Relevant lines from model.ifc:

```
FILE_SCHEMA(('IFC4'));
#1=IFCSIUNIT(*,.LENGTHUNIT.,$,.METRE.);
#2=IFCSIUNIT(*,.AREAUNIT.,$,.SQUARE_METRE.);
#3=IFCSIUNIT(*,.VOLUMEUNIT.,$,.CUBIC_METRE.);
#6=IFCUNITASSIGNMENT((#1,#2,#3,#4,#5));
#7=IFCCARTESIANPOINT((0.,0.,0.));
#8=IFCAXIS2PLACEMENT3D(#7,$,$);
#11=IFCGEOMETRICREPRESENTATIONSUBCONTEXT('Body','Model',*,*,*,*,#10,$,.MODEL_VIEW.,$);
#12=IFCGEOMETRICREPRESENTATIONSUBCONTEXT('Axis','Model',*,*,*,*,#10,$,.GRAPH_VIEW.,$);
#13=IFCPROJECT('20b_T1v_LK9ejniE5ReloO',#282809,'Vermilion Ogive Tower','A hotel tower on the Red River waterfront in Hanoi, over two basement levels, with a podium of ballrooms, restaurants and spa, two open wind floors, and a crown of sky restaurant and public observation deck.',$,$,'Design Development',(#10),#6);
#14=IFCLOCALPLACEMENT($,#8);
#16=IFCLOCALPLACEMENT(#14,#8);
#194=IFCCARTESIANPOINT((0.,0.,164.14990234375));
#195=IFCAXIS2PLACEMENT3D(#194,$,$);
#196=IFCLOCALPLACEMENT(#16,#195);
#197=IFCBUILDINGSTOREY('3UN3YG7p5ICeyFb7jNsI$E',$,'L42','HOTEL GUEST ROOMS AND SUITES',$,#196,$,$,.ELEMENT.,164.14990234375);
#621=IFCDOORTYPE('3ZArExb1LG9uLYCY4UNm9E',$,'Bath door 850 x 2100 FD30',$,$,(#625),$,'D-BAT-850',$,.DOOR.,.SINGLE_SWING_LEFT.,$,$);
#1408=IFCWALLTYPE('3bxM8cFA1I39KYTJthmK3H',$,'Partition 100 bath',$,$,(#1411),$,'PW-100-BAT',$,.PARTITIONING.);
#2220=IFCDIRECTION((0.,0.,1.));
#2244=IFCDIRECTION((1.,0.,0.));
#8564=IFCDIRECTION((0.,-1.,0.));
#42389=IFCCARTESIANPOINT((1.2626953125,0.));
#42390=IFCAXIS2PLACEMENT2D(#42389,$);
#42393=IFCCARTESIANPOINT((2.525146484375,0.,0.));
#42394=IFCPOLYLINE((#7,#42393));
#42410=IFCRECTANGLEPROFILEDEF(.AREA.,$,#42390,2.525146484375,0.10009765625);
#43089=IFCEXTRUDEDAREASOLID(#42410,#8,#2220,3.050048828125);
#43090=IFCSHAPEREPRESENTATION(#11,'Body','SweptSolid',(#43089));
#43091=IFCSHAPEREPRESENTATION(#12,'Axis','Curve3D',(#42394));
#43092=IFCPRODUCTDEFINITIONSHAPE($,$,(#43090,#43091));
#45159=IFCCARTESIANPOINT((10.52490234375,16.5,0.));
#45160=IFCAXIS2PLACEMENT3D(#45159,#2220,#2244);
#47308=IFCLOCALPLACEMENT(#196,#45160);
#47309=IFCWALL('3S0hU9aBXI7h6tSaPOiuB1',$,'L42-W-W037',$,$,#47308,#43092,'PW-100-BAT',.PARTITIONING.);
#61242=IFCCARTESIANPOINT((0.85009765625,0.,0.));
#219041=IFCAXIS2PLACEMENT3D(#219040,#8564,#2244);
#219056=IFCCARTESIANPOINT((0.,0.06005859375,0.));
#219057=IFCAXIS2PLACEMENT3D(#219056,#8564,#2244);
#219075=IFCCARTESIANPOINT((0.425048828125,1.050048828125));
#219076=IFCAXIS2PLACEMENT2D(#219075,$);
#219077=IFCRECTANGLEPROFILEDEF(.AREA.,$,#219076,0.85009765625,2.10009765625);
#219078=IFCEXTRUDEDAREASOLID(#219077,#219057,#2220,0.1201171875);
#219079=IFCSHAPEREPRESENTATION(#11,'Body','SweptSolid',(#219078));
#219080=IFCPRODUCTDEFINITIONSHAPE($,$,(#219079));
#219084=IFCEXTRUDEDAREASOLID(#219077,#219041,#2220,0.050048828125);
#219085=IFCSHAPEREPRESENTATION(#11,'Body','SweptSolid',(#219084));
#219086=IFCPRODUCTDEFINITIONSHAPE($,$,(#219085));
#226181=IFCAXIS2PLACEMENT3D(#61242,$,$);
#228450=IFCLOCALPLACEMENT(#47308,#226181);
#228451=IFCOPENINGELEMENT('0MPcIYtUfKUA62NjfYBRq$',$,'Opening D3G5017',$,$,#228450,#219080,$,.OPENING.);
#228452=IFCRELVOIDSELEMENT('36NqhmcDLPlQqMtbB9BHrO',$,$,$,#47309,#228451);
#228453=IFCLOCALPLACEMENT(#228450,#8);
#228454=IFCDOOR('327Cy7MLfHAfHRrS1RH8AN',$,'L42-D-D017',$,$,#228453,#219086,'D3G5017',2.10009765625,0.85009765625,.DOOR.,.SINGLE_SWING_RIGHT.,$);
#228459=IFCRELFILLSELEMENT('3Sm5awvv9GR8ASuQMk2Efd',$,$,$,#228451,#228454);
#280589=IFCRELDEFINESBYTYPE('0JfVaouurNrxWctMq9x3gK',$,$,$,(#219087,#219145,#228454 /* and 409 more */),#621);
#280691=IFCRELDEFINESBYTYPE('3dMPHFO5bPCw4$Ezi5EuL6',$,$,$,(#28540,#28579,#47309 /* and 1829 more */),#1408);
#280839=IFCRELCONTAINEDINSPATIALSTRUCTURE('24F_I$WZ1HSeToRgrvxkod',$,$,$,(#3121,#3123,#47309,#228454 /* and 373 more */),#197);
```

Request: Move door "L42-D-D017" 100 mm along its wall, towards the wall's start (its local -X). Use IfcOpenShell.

```python
import ifcopenshell
import ifcopenshell.api.geometry
import ifcopenshell.util.placement
import ifcopenshell.util.unit

model = ifcopenshell.open("model.ifc")
unit_scale = ifcopenshell.util.unit.calculate_unit_scale(model)

door = model.by_id(228454)
opening = door.FillsVoids[0].RelatingOpeningElement
wall = opening.VoidsElements[0].RelatingBuildingElement

wall_matrix = ifcopenshell.util.placement.get_local_placement(wall.ObjectPlacement)
shift = wall_matrix[:3, 0] * -0.1 / unit_scale
before = ifcopenshell.util.placement.get_local_placement(door.ObjectPlacement)[:3, 3].copy()

# The door is placed relative to its opening, so it follows when the opening moves.
matrix = ifcopenshell.util.placement.get_local_placement(opening.ObjectPlacement)
matrix[:3, 3] += shift
ifcopenshell.api.geometry.edit_object_placement(
    model, product=opening, matrix=matrix, is_si=False, should_transform_children=True
)

after = ifcopenshell.util.placement.get_local_placement(door.ObjectPlacement)[:3, 3]
print("door moved by", (after - before).round(3) + 0.0)

model.write("model_v2.ifc")
```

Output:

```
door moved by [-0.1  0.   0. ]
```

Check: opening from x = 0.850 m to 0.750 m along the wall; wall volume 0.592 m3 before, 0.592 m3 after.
